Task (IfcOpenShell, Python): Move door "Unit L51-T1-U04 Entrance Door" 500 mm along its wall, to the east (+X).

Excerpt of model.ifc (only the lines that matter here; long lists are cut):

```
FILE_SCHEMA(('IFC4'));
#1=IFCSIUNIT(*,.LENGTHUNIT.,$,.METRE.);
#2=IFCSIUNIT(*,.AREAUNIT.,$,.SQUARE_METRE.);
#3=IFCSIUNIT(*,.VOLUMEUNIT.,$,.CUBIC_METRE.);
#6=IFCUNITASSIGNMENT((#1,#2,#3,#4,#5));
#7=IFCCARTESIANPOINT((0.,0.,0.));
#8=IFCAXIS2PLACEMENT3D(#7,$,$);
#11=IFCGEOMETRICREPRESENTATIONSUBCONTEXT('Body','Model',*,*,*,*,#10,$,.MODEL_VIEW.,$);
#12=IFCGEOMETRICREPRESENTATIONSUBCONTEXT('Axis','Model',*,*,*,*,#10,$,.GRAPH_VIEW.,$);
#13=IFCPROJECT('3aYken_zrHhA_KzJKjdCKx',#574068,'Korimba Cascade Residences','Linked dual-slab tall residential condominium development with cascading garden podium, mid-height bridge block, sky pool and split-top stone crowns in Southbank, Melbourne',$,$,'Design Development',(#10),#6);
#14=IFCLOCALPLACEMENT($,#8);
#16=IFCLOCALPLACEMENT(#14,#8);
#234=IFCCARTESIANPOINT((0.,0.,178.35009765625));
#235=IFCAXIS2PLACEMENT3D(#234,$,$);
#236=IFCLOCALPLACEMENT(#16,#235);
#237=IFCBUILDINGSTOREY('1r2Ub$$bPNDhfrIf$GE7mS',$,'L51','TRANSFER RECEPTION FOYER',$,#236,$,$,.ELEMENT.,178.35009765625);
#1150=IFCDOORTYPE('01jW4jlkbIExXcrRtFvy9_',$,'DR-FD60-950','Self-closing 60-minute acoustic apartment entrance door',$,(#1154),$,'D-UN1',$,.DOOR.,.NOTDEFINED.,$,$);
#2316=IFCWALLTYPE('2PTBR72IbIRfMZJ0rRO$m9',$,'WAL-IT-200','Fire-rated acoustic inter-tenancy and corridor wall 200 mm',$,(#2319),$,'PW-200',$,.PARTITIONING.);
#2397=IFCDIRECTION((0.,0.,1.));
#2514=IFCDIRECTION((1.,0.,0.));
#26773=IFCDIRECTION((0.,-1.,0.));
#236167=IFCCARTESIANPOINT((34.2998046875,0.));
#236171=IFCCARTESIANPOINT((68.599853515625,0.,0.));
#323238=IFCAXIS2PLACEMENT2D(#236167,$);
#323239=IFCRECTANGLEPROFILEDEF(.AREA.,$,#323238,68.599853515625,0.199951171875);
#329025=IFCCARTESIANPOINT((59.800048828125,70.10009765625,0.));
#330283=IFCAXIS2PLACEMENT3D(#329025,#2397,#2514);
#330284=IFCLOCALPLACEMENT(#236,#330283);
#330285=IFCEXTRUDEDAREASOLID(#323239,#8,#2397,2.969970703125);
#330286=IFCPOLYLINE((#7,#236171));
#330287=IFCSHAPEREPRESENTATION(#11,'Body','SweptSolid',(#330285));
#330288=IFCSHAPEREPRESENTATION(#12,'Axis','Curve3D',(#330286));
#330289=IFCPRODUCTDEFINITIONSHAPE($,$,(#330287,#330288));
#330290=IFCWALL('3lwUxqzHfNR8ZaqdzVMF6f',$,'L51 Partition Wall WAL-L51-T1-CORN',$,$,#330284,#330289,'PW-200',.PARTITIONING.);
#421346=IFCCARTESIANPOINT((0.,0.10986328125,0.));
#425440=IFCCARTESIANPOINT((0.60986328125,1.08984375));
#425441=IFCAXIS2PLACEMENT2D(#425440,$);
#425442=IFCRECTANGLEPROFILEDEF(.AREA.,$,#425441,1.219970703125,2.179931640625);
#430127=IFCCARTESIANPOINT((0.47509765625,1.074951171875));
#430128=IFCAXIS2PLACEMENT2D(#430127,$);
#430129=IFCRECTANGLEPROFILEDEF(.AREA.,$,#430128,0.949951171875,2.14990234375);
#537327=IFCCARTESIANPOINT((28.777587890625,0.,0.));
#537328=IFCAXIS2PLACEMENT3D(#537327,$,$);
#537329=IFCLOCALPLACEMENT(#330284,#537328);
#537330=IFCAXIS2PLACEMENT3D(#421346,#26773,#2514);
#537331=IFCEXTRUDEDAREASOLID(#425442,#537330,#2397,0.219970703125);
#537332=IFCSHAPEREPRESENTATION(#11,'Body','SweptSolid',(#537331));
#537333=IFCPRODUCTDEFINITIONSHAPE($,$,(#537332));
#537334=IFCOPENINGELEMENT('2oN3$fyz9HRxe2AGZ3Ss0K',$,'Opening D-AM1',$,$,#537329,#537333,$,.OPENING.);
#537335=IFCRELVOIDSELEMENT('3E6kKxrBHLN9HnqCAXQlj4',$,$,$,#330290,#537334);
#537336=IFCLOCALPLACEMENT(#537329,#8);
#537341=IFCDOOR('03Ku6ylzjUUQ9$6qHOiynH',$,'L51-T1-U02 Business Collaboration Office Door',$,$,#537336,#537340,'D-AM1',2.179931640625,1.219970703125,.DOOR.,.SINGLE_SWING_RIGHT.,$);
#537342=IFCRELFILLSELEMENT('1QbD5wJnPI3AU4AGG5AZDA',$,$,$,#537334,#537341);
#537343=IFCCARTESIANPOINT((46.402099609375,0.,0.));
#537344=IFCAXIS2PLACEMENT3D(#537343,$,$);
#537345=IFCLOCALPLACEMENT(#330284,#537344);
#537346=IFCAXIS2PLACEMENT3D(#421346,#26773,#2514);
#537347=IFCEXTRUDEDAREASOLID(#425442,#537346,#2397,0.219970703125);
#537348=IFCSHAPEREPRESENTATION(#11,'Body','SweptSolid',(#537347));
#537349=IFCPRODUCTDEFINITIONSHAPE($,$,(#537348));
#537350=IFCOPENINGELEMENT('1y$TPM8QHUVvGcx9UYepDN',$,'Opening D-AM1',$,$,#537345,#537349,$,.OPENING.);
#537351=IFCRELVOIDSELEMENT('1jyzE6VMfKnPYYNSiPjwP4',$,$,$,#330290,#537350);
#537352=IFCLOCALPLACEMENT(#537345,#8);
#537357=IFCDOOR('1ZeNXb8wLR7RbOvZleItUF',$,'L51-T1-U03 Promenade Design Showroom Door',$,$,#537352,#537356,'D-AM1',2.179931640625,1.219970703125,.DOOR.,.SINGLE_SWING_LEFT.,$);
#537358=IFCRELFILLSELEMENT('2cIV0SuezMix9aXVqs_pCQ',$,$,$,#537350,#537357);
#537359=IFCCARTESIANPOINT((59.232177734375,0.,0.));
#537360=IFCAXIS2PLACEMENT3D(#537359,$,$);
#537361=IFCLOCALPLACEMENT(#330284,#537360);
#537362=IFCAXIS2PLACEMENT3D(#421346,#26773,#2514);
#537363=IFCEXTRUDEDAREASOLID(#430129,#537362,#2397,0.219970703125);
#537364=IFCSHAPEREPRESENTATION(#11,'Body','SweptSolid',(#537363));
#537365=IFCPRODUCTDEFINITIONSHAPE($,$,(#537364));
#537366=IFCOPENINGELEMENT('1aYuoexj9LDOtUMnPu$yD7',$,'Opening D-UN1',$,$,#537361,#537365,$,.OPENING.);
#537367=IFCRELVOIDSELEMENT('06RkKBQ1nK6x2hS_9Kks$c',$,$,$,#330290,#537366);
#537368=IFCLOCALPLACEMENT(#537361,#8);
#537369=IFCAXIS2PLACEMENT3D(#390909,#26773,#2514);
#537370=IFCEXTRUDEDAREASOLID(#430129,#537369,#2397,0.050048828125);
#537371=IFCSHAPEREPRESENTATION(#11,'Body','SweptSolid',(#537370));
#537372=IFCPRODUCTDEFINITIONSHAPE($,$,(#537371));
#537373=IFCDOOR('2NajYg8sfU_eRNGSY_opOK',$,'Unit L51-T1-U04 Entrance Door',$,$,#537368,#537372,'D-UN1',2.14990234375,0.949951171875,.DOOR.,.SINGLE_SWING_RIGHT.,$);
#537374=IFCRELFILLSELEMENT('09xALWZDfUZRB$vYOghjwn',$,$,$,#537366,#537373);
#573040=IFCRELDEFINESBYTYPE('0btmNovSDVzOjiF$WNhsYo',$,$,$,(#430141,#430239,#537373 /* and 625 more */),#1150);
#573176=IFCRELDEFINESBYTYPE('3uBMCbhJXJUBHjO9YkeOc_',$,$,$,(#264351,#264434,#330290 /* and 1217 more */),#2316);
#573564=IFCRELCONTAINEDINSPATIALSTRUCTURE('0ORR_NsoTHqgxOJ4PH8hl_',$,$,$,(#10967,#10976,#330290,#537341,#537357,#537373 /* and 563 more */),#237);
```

```python
import ifcopenshell
import ifcopenshell.api.geometry
import ifcopenshell.util.placement
import ifcopenshell.util.unit

model = ifcopenshell.open("model.ifc")
unit_scale = ifcopenshell.util.unit.calculate_unit_scale(model)

door = model.by_guid("2NajYg8sfU_eRNGSY_opOK")
opening = door.FillsVoids[0].RelatingOpeningElement
wall = opening.VoidsElements[0].RelatingBuildingElement

wall_matrix = ifcopenshell.util.placement.get_local_placement(wall.ObjectPlacement)
shift = wall_matrix[:3, 0] * 0.5 / unit_scale
before = ifcopenshell.util.placement.get_local_placement(door.ObjectPlacement)[:3, 3].copy()

# The door is placed relative to its opening, so it follows when the opening moves.
matrix = ifcopenshell.util.placement.get_local_placement(opening.ObjectPlacement)
matrix[:3, 3] += shift
ifcopenshell.api.geometry.edit_object_placement(
    model, product=opening, matrix=matrix, is_si=False, should_transform_children=True
)

after = ifcopenshell.util.placement.get_local_placement(door.ObjectPlacement)[:3, 3]
print("door moved by", (after - before).round(3) + 0.0)

model.write("model_edited.ifc")
```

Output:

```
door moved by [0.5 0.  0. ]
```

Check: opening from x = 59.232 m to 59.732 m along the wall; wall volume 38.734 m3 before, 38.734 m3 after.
